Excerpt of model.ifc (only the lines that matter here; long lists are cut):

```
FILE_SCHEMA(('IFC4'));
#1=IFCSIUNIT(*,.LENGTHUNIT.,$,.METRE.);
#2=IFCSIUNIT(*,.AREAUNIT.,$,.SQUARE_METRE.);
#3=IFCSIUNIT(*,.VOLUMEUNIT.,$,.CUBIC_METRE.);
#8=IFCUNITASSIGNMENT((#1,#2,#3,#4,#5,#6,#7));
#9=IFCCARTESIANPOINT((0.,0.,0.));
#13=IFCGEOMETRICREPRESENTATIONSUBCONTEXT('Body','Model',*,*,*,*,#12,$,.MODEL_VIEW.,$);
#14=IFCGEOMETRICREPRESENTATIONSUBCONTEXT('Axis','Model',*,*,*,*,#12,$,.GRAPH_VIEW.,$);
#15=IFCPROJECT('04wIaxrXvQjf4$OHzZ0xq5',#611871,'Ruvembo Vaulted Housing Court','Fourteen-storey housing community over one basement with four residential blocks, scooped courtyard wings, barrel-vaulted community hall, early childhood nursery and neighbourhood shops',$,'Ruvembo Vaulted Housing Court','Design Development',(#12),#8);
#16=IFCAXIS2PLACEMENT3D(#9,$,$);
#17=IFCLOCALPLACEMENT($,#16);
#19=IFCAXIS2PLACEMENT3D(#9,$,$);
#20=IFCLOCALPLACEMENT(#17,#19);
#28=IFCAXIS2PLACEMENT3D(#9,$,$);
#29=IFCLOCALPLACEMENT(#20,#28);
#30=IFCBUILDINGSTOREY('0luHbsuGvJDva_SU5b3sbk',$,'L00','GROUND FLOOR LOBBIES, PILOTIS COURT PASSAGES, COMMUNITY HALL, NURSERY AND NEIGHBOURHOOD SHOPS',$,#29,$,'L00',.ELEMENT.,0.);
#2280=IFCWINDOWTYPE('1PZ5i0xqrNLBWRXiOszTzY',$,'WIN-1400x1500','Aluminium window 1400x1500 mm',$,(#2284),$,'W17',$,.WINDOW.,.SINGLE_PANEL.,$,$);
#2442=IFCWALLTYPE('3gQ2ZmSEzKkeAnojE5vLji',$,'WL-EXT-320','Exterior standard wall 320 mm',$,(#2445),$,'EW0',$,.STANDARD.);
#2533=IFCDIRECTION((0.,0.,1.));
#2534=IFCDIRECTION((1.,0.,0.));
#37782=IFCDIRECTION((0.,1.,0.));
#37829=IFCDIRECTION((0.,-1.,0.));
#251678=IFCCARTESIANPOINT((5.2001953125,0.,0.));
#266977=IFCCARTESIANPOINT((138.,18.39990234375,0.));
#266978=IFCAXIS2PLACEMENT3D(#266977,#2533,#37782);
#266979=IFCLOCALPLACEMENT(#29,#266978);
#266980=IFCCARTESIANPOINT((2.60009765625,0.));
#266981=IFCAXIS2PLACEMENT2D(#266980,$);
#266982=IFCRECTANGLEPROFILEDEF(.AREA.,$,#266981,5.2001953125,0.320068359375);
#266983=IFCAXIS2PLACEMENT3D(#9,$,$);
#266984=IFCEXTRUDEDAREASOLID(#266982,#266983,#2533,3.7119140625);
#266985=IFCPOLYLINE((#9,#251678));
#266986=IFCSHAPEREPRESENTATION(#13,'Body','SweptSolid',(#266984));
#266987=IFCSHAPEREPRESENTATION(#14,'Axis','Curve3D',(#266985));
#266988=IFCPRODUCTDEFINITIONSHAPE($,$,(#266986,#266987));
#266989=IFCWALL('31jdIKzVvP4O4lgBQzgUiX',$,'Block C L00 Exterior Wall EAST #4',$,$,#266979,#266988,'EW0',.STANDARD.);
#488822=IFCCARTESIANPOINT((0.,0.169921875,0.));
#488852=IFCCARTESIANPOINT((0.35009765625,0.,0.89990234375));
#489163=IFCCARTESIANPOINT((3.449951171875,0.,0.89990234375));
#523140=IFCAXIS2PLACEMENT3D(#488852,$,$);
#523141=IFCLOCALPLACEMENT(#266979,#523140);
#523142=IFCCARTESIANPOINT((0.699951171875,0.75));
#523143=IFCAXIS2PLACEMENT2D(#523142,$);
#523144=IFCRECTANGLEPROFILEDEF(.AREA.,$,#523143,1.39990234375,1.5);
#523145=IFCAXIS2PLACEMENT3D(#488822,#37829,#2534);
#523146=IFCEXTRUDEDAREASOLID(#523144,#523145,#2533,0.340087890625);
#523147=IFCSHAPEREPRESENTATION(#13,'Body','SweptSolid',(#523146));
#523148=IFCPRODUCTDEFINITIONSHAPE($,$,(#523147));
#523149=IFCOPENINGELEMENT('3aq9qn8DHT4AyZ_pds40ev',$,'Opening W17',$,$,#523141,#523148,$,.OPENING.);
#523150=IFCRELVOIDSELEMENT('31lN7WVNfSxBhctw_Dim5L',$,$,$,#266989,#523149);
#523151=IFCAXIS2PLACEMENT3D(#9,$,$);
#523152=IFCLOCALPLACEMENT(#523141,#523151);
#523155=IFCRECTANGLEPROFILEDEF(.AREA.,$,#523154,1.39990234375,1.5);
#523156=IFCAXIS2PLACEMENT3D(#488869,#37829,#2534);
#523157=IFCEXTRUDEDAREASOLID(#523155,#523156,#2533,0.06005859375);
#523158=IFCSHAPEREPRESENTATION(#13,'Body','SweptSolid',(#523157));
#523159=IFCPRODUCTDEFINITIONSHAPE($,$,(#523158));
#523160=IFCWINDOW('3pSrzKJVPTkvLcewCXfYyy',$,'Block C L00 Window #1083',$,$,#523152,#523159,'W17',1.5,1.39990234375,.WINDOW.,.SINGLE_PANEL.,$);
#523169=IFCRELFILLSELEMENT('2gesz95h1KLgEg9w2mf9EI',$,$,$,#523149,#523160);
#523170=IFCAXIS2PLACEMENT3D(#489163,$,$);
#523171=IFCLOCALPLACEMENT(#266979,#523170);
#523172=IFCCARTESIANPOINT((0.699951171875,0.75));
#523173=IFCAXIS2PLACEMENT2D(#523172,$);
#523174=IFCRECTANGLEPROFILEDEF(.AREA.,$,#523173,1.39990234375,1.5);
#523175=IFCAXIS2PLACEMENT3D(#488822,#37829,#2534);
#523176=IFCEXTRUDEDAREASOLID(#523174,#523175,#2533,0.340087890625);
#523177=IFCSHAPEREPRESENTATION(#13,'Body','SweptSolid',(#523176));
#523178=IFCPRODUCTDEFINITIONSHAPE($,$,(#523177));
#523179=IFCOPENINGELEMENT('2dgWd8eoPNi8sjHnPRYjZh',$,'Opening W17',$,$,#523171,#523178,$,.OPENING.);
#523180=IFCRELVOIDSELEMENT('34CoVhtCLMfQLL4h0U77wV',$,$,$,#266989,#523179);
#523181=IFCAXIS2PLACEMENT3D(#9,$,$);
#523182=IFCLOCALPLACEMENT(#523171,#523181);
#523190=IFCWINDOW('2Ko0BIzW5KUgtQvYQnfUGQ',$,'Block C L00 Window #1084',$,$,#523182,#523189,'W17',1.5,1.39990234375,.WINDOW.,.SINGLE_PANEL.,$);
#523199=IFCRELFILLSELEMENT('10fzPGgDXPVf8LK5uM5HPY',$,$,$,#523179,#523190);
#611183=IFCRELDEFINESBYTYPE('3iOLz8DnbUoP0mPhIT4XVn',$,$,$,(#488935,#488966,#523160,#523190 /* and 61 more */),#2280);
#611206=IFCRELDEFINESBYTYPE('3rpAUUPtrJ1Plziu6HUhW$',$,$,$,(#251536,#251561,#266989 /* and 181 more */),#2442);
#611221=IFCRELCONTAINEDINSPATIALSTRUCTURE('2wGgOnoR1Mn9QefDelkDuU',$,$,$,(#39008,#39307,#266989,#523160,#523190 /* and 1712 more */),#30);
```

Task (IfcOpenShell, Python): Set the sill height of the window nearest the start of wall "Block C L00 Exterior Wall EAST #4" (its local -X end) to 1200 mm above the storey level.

```python
import numpy as np
import ifcopenshell
import ifcopenshell.api.geometry
import ifcopenshell.geom
import ifcopenshell.util.element
import ifcopenshell.util.placement
import ifcopenshell.util.shape
import ifcopenshell.util.unit

model = ifcopenshell.open("model.ifc")
unit_scale = ifcopenshell.util.unit.calculate_unit_scale(model)

window = model.by_guid("3pSrzKJVPTkvLcewCXfYyy")
opening = window.FillsVoids[0].RelatingOpeningElement
storey = ifcopenshell.util.element.get_container(window, ifc_class="IfcBuildingStorey")
level = ifcopenshell.util.placement.get_local_placement(storey.ObjectPlacement)[2, 3]

# The opening's origin need not be at the sill, so measure its lowest point.
shape = ifcopenshell.geom.create_shape(ifcopenshell.geom.settings(), opening)
bottom = ifcopenshell.util.shape.get_shape_bottom_elevation(shape, shape.geometry) / unit_scale
dz = level + 1.2 / unit_scale - bottom

shift = np.array([0.0, 0.0, dz])
# The window is placed relative to its opening, so it follows when the opening moves.
matrix = ifcopenshell.util.placement.get_local_placement(opening.ObjectPlacement)
matrix[:3, 3] += shift
ifcopenshell.api.geometry.edit_object_placement(
    model, product=opening, matrix=matrix, is_si=False, should_transform_children=True
)

print(f"moved by {dz * unit_scale:+.3f} m")

model.write("model-out.ifc")
```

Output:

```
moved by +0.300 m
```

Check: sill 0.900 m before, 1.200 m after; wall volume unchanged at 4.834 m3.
